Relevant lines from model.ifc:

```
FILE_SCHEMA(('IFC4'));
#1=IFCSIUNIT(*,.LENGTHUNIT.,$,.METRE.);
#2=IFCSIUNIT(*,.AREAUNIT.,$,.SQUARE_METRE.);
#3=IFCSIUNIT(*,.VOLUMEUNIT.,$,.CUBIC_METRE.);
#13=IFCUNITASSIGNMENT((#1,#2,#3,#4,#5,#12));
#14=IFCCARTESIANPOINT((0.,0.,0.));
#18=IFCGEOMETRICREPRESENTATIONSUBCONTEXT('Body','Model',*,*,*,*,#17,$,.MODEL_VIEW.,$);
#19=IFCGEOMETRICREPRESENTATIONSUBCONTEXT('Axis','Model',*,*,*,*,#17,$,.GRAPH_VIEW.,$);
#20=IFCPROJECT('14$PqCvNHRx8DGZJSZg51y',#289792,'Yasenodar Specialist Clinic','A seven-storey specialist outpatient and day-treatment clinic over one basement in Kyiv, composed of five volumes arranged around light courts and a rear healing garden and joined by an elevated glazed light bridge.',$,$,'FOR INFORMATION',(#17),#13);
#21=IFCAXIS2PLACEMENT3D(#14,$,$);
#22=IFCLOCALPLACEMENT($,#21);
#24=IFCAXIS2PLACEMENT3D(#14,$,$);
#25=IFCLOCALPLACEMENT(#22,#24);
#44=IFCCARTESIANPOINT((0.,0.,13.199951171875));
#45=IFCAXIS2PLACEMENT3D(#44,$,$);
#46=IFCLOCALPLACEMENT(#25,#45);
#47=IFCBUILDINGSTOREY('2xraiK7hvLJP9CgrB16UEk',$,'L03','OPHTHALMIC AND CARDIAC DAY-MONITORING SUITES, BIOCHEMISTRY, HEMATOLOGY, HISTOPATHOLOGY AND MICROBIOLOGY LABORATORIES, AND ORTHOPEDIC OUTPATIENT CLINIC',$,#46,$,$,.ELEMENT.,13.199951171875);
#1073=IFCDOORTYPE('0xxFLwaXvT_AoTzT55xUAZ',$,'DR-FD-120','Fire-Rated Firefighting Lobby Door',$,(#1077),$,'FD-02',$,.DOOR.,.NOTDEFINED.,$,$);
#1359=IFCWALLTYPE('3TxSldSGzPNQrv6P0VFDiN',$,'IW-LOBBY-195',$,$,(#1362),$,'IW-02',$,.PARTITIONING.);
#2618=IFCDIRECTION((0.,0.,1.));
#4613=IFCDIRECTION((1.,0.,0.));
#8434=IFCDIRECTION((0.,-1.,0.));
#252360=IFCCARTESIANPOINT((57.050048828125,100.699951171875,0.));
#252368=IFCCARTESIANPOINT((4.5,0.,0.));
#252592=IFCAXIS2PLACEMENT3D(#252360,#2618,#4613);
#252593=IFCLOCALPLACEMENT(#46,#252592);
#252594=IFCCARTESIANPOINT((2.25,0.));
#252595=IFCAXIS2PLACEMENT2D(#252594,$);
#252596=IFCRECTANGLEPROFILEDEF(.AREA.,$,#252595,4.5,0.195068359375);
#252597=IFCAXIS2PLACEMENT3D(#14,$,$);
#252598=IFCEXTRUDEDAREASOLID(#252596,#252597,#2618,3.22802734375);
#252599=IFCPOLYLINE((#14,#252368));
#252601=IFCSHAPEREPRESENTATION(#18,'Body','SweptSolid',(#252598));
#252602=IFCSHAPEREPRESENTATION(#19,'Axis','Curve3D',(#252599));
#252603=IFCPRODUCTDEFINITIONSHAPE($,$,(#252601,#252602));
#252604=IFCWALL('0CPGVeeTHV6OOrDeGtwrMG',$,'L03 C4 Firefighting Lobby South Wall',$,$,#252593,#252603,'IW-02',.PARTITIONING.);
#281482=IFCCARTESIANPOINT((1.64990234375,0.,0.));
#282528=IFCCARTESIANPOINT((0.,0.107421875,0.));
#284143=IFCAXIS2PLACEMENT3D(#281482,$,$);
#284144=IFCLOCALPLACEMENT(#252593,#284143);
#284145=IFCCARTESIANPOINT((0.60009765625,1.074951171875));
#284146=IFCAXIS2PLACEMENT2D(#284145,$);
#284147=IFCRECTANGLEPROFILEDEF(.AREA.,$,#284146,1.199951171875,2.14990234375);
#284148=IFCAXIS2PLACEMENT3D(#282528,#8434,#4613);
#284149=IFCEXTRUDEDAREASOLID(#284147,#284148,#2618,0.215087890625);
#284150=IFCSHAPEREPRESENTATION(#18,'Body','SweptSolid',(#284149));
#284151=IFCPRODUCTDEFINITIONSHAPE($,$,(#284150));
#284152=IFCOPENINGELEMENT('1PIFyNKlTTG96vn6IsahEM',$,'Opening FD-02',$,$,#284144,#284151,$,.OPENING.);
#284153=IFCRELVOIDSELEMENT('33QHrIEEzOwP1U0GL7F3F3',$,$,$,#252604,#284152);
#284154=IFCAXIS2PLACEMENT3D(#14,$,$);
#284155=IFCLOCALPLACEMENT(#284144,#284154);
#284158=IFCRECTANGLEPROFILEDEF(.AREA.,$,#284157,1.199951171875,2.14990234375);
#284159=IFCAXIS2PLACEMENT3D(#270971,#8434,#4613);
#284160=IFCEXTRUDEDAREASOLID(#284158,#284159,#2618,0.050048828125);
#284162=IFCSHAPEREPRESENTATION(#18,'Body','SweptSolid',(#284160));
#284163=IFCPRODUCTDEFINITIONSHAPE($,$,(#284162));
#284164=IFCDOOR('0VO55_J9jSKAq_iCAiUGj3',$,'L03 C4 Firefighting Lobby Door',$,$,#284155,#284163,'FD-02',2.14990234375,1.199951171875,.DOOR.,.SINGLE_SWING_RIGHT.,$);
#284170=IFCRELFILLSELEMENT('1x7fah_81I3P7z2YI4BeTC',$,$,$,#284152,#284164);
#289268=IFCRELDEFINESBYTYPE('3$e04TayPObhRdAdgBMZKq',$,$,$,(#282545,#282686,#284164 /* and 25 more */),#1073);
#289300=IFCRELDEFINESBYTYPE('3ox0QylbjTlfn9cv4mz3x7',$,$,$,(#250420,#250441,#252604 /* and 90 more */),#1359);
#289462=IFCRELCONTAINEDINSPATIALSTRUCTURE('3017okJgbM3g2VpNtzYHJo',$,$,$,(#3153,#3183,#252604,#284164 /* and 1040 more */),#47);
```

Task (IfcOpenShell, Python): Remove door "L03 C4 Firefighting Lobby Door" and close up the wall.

```python
import ifcopenshell
import ifcopenshell.api.feature
import ifcopenshell.api.root
import ifcopenshell.geom
import ifcopenshell.util.shape

model = ifcopenshell.open("model.ifc")
settings = ifcopenshell.geom.settings()


def volume(element):
    """Net volume in cubic metres, openings subtracted."""
    shape = ifcopenshell.geom.create_shape(settings, element)
    return ifcopenshell.util.shape.get_volume(shape.geometry)


door = model.by_guid("0VO55_J9jSKAq_iCAiUGj3")
opening = door.FillsVoids[0].RelatingOpeningElement
wall = opening.VoidsElements[0].RelatingBuildingElement
before = volume(wall)

ifcopenshell.api.root.remove_product(model, product=door)
ifcopenshell.api.feature.remove_feature(model, feature=opening)

after = volume(wall)

print(f"wall volume {before:.3f} -> {after:.3f} m3")

model.write("model_v2.ifc")
```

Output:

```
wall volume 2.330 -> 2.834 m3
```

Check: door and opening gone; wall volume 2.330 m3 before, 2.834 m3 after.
